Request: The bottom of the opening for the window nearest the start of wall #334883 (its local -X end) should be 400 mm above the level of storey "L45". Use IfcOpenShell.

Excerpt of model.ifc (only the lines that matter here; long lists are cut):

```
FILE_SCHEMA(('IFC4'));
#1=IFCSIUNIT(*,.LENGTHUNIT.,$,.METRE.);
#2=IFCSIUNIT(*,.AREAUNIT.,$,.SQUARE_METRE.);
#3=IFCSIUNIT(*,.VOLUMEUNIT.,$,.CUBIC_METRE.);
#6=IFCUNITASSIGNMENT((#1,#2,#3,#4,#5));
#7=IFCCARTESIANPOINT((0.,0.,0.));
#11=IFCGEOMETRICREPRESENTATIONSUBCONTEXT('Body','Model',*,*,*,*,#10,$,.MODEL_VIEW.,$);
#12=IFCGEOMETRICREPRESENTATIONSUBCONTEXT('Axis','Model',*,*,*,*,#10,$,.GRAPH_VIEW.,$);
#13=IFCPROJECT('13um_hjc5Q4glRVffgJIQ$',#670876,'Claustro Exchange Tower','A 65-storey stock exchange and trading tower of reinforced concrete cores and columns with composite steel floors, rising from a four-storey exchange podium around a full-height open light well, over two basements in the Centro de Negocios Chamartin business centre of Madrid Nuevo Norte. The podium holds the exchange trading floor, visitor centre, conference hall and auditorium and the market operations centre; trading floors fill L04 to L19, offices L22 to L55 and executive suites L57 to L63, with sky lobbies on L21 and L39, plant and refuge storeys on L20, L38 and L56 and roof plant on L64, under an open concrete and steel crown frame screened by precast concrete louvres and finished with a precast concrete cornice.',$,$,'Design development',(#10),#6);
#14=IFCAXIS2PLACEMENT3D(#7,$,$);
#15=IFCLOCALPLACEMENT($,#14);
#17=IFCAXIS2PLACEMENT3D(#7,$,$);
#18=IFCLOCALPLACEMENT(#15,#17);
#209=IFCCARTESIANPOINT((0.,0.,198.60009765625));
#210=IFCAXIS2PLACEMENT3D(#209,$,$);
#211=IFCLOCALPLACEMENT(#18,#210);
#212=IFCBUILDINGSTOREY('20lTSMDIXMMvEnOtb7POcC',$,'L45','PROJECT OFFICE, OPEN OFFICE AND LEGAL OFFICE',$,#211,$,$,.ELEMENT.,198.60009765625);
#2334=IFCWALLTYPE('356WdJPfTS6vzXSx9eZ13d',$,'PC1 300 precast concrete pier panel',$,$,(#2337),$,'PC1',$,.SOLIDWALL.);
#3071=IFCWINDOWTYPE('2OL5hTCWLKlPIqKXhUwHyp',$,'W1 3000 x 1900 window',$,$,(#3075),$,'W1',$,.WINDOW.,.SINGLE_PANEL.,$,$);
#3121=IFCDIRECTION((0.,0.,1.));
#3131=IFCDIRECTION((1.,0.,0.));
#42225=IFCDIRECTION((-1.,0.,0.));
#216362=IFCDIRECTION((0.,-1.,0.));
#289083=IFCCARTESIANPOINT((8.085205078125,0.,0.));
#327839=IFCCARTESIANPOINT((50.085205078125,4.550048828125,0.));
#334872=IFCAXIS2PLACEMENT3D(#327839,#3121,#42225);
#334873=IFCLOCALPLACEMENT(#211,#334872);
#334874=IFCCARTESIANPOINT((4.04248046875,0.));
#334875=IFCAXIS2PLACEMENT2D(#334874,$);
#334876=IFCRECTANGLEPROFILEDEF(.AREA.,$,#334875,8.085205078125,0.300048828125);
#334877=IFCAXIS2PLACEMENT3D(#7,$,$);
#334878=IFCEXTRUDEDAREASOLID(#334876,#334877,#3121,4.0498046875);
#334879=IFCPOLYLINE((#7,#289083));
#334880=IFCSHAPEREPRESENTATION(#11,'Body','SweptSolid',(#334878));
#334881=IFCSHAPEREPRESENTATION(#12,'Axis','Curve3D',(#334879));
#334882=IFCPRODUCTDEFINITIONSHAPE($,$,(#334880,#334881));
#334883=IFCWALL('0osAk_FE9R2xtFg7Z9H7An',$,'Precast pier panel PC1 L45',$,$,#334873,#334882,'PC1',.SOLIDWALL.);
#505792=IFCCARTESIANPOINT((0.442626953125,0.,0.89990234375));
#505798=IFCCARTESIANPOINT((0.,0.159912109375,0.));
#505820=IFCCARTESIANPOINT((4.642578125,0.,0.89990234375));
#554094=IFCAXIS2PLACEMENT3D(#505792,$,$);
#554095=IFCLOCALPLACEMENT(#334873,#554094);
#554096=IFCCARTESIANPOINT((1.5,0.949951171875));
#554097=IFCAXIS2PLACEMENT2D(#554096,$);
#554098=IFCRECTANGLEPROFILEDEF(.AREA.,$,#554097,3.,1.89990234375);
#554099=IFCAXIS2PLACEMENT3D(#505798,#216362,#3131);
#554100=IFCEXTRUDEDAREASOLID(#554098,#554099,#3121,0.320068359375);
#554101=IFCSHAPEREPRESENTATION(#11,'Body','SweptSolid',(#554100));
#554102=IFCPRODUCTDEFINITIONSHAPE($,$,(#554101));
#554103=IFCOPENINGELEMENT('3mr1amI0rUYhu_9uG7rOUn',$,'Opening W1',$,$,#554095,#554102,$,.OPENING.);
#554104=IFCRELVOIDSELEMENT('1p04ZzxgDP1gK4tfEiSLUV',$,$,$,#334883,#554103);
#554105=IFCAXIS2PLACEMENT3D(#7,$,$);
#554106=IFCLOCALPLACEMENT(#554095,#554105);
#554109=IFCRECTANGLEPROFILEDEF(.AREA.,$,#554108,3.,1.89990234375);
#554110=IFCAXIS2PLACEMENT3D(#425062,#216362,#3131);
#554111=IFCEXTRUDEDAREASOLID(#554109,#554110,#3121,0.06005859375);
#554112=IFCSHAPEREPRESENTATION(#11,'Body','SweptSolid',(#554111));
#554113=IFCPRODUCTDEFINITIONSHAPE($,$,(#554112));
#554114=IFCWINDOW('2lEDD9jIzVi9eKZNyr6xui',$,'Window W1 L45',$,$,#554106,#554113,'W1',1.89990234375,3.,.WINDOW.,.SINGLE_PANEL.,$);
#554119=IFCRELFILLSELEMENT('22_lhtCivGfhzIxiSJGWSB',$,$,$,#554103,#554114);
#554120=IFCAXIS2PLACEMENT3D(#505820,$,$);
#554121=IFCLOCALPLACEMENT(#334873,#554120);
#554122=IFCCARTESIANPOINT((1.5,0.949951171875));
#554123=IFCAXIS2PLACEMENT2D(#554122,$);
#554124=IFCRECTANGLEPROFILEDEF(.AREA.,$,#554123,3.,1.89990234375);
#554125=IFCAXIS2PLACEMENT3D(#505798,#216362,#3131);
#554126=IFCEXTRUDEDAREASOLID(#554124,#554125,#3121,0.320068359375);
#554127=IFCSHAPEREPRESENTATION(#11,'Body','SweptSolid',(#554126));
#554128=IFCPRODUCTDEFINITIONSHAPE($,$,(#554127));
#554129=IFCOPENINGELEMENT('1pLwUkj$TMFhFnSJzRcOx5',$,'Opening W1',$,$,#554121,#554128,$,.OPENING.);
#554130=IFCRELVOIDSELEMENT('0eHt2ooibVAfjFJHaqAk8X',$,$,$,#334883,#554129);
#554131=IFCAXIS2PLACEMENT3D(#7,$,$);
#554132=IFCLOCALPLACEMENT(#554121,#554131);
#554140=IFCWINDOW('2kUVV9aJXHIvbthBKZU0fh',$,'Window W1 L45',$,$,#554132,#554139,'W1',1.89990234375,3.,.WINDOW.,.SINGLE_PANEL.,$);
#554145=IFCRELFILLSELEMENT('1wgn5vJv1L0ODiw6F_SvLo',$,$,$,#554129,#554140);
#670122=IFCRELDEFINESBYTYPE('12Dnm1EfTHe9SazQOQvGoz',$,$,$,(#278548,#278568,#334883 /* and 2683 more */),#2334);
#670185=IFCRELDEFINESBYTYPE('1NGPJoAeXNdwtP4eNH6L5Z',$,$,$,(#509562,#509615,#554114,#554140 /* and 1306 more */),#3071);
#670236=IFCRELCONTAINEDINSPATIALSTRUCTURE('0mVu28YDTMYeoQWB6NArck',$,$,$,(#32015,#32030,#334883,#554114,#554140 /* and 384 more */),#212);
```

```python
import numpy as np
import ifcopenshell
import ifcopenshell.api.geometry
import ifcopenshell.geom
import ifcopenshell.util.element
import ifcopenshell.util.placement
import ifcopenshell.util.shape
import ifcopenshell.util.unit

model = ifcopenshell.open("model.ifc")
unit_scale = ifcopenshell.util.unit.calculate_unit_scale(model)

window = model.by_guid("2lEDD9jIzVi9eKZNyr6xui")
opening = window.FillsVoids[0].RelatingOpeningElement
storey = ifcopenshell.util.element.get_container(window, ifc_class="IfcBuildingStorey")
level = ifcopenshell.util.placement.get_local_placement(storey.ObjectPlacement)[2, 3]

# The opening's origin need not be at the sill, so measure its lowest point.
shape = ifcopenshell.geom.create_shape(ifcopenshell.geom.settings(), opening)
bottom = ifcopenshell.util.shape.get_shape_bottom_elevation(shape, shape.geometry) / unit_scale
dz = level + 0.4 / unit_scale - bottom

shift = np.array([0.0, 0.0, dz])
# The window is placed relative to its opening, so it follows when the opening moves.
matrix = ifcopenshell.util.placement.get_local_placement(opening.ObjectPlacement)
matrix[:3, 3] += shift
ifcopenshell.api.geometry.edit_object_placement(
    model, product=opening, matrix=matrix, is_si=False, should_transform_children=True
)

print(f"moved by {dz * unit_scale:+.3f} m")

model.write("model_rev.ifc")
```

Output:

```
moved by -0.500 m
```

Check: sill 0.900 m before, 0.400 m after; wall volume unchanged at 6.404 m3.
